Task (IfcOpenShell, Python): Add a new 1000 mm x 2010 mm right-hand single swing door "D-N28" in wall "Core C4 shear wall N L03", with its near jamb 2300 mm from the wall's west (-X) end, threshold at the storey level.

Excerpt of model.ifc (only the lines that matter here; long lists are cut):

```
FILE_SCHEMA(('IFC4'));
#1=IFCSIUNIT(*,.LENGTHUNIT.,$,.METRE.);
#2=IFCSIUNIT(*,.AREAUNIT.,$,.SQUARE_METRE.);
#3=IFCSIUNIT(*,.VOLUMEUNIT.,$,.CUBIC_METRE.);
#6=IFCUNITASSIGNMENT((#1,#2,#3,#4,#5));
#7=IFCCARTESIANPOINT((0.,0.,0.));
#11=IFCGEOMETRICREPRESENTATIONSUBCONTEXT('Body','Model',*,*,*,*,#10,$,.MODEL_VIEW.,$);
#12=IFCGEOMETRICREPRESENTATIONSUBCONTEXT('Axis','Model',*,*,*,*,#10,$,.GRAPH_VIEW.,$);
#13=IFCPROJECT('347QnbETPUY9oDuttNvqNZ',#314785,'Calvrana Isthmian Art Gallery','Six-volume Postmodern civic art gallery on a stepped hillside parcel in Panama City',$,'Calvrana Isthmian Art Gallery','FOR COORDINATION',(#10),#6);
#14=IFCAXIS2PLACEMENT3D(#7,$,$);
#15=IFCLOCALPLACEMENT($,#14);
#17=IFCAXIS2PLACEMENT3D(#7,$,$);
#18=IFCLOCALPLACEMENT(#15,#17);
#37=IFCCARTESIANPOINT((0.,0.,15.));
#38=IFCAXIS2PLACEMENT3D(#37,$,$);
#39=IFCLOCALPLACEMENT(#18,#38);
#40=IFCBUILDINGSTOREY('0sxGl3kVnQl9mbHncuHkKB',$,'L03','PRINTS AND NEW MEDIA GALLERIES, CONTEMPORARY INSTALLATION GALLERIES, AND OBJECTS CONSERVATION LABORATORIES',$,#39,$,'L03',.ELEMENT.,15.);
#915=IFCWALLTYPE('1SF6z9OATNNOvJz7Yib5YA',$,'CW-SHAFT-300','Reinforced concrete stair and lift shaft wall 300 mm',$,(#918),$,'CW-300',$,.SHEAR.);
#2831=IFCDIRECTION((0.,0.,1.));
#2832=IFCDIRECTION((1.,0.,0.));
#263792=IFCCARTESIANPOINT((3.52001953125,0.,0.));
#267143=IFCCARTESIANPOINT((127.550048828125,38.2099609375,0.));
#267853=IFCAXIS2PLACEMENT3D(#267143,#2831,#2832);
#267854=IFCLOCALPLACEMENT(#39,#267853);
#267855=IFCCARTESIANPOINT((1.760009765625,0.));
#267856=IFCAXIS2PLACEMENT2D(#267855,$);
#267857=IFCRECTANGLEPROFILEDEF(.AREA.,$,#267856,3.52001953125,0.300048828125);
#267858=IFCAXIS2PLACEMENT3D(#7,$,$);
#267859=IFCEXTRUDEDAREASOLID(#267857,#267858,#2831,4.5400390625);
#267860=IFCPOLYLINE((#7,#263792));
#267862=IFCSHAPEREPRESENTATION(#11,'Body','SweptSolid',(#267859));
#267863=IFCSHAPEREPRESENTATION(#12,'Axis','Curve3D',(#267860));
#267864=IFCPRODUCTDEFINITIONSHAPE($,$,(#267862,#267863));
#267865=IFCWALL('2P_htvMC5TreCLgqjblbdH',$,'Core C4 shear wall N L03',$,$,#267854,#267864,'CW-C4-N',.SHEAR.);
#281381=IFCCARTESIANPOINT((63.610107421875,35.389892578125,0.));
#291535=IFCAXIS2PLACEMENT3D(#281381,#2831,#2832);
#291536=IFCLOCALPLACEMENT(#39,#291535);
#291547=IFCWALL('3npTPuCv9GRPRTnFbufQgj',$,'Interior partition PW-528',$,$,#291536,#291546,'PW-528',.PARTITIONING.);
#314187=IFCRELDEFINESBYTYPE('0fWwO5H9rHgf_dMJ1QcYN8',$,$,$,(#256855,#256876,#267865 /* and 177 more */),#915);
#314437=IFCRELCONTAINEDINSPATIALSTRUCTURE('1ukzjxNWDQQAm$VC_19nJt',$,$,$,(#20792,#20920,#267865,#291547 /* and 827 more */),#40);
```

```python
import numpy as np
import ifcopenshell
import ifcopenshell.api.feature
import ifcopenshell.api.geometry
import ifcopenshell.api.root
import ifcopenshell.api.spatial
import ifcopenshell.geom
import ifcopenshell.util.element
import ifcopenshell.util.placement
import ifcopenshell.util.representation
import ifcopenshell.util.shape
import ifcopenshell.util.unit

model = ifcopenshell.open("model.ifc")
unit_scale = ifcopenshell.util.unit.calculate_unit_scale(model)
settings = ifcopenshell.geom.settings()


def volume(element):
    """Net volume in cubic metres, openings subtracted."""
    shape = ifcopenshell.geom.create_shape(settings, element)
    return ifcopenshell.util.shape.get_volume(shape.geometry)


wall = model.by_guid("2P_htvMC5TreCLgqjblbdH")
storey = ifcopenshell.util.element.get_container(wall, ifc_class="IfcBuildingStorey")
context = ifcopenshell.util.representation.get_context(model, "Model", "Body", "MODEL_VIEW")
before = volume(wall)

width, height, from_end, sill = 1, 2.01, 2.3, 0.0  # metres

# The wall runs along its own X axis, and the end named is its -X end.
wall_shape = ifcopenshell.geom.create_shape(settings, wall)
x, y, z = ifcopenshell.util.shape.get_vertices(wall_shape.geometry).T
start = x.min() + from_end
face, thickness = float(y.min()), float(y.max() - y.min())
wall_matrix = ifcopenshell.util.placement.get_local_placement(wall.ObjectPlacement)
level = ifcopenshell.util.placement.get_local_placement(storey.ObjectPlacement)[2, 3]


def in_wall(x, y):
    """Placement at x, y metres in the wall's axes, at sill height."""
    matrix = wall_matrix.copy()
    matrix[:, 3] = wall_matrix @ np.array([x / unit_scale, y / unit_scale, 0.0, 1.0])
    matrix[2, 3] = level + sill / unit_scale
    return matrix


# Opening: a box that overshoots both wall faces by 50 mm.
opening = ifcopenshell.api.root.create_entity(model, ifc_class="IfcOpeningElement", predefined_type="OPENING")
box = ifcopenshell.api.geometry.add_wall_representation(
    model, context=context, length=width, height=height, thickness=thickness + 0.1
)
ifcopenshell.api.geometry.assign_representation(model, product=opening, representation=box)
ifcopenshell.api.geometry.edit_object_placement(model, product=opening, matrix=in_wall(start, face - 0.05), is_si=False)
ifcopenshell.api.feature.add_feature(model, feature=opening, element=wall)

door = ifcopenshell.api.root.create_entity(model, ifc_class="IfcDoor", name="D-N28", predefined_type="DOOR")
door.OverallWidth, door.OverallHeight = width / unit_scale, height / unit_scale
door.OperationType = "SINGLE_SWING_RIGHT"
body = ifcopenshell.api.geometry.add_door_representation(
    model,
    context=context,
    overall_width=door.OverallWidth,
    overall_height=door.OverallHeight,
    operation_type="SINGLE_SWING_RIGHT",
    lining_properties={"LiningDepth": thickness / unit_scale, "ThresholdDepth": thickness / unit_scale},
)
ifcopenshell.api.geometry.assign_representation(model, product=door, representation=body)
ifcopenshell.api.spatial.assign_container(model, products=[door], relating_structure=storey)
ifcopenshell.api.feature.add_filling(model, opening=opening, element=door)

# The lining spans the wall, so the door starts at the wall face.
ifcopenshell.api.geometry.edit_object_placement(model, product=door, matrix=in_wall(start, face), is_si=False)

after = volume(wall)

print(f"wall volume {before:.3f} -> {after:.3f} m3")

model.write("model_v2.ifc")
```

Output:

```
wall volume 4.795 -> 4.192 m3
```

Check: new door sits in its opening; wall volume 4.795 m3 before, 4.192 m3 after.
